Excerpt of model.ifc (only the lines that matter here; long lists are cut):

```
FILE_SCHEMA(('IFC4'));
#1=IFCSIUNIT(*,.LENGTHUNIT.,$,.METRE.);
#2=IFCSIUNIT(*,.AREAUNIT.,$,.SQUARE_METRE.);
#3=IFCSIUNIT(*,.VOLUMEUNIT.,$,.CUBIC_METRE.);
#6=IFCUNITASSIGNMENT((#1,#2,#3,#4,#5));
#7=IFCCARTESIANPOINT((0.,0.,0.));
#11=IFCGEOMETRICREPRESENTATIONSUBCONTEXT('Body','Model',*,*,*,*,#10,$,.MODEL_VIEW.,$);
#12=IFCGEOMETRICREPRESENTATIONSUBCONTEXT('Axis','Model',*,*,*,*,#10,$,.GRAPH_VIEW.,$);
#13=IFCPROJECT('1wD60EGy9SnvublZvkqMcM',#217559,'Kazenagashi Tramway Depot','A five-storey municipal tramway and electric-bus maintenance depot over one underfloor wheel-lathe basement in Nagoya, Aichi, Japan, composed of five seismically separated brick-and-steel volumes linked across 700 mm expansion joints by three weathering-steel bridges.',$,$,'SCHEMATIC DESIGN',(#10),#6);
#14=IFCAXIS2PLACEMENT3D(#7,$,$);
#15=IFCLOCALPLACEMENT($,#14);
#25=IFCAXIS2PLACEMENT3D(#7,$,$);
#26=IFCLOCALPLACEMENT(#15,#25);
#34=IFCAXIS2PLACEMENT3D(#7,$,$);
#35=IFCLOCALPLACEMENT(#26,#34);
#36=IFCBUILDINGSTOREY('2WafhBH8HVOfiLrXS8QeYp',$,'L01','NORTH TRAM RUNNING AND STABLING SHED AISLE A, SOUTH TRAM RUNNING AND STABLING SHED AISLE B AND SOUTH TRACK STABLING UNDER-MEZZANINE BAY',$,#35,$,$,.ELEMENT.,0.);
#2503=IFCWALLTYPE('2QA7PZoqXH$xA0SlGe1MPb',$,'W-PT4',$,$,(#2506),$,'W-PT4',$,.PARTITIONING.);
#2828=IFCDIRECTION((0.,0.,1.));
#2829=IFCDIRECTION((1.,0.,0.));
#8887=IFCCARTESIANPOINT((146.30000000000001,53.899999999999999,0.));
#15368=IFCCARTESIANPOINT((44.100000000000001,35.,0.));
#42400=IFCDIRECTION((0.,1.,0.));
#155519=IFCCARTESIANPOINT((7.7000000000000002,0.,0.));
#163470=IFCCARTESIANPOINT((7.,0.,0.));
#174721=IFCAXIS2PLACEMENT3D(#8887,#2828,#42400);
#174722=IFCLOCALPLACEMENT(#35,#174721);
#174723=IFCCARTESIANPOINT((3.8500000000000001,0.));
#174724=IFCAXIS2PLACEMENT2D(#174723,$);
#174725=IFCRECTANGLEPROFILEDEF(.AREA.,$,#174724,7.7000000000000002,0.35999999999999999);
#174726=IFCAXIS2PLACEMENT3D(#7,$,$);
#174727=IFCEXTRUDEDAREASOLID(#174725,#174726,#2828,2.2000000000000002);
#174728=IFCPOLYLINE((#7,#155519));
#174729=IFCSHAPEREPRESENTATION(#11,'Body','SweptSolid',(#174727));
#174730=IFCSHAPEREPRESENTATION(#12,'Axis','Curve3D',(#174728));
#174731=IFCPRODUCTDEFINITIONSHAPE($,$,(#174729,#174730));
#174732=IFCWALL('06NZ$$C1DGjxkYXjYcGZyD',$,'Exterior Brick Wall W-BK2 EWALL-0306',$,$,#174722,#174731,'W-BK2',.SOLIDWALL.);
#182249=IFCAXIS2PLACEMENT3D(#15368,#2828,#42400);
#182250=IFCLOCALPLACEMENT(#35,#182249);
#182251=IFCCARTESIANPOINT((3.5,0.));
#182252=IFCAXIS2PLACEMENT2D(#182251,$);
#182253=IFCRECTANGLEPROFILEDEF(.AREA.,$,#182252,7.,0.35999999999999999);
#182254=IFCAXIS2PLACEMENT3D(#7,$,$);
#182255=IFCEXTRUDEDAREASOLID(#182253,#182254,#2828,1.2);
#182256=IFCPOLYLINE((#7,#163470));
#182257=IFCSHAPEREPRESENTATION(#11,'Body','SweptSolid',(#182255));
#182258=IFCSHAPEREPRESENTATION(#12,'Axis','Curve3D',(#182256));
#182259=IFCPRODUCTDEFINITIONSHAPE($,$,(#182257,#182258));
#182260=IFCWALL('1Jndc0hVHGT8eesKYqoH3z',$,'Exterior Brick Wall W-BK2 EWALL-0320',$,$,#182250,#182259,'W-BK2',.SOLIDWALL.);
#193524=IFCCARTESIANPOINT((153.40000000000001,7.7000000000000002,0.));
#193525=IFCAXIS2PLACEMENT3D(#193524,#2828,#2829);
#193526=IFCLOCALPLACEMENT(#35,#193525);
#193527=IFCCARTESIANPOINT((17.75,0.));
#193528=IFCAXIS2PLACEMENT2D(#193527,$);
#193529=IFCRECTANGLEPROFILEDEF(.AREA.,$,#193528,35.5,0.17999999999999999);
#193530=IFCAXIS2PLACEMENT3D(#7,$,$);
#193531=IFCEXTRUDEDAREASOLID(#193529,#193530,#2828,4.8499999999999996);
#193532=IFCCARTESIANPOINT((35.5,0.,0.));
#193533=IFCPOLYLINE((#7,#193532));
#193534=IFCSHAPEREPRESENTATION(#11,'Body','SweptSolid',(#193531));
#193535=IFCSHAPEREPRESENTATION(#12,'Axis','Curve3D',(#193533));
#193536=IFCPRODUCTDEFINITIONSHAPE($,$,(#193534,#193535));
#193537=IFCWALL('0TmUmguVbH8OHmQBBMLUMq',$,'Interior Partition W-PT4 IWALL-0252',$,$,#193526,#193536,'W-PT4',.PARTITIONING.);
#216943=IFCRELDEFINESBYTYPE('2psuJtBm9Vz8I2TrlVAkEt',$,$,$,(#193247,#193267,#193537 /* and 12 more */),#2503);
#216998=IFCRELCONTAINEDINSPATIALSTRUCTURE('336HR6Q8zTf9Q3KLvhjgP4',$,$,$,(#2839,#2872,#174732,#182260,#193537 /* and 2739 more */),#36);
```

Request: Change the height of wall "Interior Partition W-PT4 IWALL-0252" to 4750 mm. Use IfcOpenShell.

```python
import ifcopenshell
import ifcopenshell.geom
import ifcopenshell.util.representation
import ifcopenshell.util.shape

model = ifcopenshell.open("model.ifc")
settings = ifcopenshell.geom.settings()


def volume(element):
    """Net volume in cubic metres, openings subtracted."""
    shape = ifcopenshell.geom.create_shape(settings, element)
    return ifcopenshell.util.shape.get_volume(shape.geometry)


wall = model.by_guid("0TmUmguVbH8OHmQBBMLUMq")
before = volume(wall)

body = ifcopenshell.util.representation.get_representation(wall, "Model", "Body")
solid = body.Items[0]
old_height = solid.Depth
solid.Depth = 4.75
after = volume(wall)

print(f"height {old_height:g} -> {solid.Depth:g}, volume {before:.3f} -> {after:.3f} m3")

model.write("model_edited.ifc")
```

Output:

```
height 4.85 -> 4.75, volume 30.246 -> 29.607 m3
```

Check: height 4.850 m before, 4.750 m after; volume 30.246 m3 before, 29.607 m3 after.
